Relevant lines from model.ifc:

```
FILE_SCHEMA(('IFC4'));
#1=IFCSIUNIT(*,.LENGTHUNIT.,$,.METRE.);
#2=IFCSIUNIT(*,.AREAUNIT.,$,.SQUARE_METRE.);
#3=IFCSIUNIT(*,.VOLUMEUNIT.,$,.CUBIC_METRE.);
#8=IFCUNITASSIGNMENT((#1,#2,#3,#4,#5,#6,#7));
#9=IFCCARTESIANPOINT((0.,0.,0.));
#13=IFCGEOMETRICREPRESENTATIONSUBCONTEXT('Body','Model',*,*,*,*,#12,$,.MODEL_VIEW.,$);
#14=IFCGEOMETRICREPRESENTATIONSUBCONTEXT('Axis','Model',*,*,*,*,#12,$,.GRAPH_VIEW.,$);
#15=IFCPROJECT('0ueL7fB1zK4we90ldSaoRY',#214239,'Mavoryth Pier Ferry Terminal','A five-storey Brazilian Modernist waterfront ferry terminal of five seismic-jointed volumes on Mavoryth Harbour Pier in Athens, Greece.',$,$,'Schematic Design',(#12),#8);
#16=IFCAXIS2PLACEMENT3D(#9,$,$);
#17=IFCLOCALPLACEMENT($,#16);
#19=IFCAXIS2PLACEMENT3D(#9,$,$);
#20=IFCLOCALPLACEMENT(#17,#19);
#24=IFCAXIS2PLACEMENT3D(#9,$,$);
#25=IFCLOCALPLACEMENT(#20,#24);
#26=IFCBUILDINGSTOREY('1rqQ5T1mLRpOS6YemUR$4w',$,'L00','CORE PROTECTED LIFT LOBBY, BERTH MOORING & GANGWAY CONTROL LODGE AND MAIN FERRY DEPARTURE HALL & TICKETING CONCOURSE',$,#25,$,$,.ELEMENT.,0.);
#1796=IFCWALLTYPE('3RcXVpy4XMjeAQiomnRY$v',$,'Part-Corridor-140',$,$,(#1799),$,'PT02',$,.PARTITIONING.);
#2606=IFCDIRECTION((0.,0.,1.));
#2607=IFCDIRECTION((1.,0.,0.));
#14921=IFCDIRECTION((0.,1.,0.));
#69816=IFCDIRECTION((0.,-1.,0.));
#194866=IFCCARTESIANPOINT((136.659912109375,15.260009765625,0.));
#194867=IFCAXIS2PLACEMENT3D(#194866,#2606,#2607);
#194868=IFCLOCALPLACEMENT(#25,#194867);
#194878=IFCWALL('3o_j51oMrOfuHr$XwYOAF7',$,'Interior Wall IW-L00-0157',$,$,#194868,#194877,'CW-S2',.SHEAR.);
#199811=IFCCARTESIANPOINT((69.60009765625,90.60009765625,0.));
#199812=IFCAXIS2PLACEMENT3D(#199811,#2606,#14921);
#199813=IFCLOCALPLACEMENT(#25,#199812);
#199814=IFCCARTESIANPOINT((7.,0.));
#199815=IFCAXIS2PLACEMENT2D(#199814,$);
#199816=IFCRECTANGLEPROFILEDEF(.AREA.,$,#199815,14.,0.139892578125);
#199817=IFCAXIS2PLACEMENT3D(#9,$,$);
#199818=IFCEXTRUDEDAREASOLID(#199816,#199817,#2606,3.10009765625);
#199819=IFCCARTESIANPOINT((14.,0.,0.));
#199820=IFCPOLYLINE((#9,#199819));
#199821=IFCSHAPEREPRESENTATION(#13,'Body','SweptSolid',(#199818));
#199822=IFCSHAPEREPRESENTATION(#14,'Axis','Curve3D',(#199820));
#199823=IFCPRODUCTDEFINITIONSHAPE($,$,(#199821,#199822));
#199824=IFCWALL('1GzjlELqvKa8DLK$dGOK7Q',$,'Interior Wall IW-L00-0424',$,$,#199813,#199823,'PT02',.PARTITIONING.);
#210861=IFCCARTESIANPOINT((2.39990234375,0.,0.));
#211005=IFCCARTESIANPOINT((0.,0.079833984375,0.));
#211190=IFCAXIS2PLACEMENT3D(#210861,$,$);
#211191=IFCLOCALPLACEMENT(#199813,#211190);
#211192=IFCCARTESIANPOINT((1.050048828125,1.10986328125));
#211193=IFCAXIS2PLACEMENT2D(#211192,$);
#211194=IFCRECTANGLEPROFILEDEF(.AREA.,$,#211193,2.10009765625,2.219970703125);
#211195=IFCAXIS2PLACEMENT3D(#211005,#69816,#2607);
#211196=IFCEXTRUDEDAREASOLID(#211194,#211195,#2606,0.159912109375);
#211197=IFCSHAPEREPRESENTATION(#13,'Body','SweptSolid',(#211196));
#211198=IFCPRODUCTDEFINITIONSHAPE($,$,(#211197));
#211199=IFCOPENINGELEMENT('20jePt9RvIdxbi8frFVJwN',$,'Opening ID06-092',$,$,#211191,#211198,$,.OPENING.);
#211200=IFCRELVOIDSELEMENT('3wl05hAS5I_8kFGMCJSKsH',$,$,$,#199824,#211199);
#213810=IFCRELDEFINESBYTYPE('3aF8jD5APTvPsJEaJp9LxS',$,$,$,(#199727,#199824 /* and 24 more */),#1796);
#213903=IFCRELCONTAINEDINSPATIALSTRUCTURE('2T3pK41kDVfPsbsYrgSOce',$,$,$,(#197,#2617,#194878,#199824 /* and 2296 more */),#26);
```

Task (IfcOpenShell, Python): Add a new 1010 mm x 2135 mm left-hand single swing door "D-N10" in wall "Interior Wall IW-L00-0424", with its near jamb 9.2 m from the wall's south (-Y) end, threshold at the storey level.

```python
import numpy as np
import ifcopenshell
import ifcopenshell.api.feature
import ifcopenshell.api.geometry
import ifcopenshell.api.root
import ifcopenshell.api.spatial
import ifcopenshell.geom
import ifcopenshell.util.element
import ifcopenshell.util.placement
import ifcopenshell.util.representation
import ifcopenshell.util.shape
import ifcopenshell.util.unit

model = ifcopenshell.open("model.ifc")
unit_scale = ifcopenshell.util.unit.calculate_unit_scale(model)
settings = ifcopenshell.geom.settings()


def volume(element):
    """Net volume in cubic metres, openings subtracted."""
    shape = ifcopenshell.geom.create_shape(settings, element)
    return ifcopenshell.util.shape.get_volume(shape.geometry)


wall = model.by_guid("1GzjlELqvKa8DLK$dGOK7Q")
storey = ifcopenshell.util.element.get_container(wall, ifc_class="IfcBuildingStorey")
context = ifcopenshell.util.representation.get_context(model, "Model", "Body", "MODEL_VIEW")
before = volume(wall)

width, height, from_end, sill = 1.01, 2.135, 9.2, 0.0  # metres

# The wall runs along its own X axis, and the end named is its -X end.
wall_shape = ifcopenshell.geom.create_shape(settings, wall)
x, y, z = ifcopenshell.util.shape.get_vertices(wall_shape.geometry).T
start = x.min() + from_end
face, thickness = float(y.min()), float(y.max() - y.min())
wall_matrix = ifcopenshell.util.placement.get_local_placement(wall.ObjectPlacement)
level = ifcopenshell.util.placement.get_local_placement(storey.ObjectPlacement)[2, 3]


def in_wall(x, y):
    """Placement at x, y metres in the wall's axes, at sill height."""
    matrix = wall_matrix.copy()
    matrix[:, 3] = wall_matrix @ np.array([x / unit_scale, y / unit_scale, 0.0, 1.0])
    matrix[2, 3] = level + sill / unit_scale
    return matrix


# Opening: a box that overshoots both wall faces by 50 mm.
opening = ifcopenshell.api.root.create_entity(model, ifc_class="IfcOpeningElement", predefined_type="OPENING")
box = ifcopenshell.api.geometry.add_wall_representation(
    model, context=context, length=width, height=height, thickness=thickness + 0.1
)
ifcopenshell.api.geometry.assign_representation(model, product=opening, representation=box)
ifcopenshell.api.geometry.edit_object_placement(model, product=opening, matrix=in_wall(start, face - 0.05), is_si=False)
ifcopenshell.api.feature.add_feature(model, feature=opening, element=wall)

door = ifcopenshell.api.root.create_entity(model, ifc_class="IfcDoor", name="D-N10", predefined_type="DOOR")
door.OverallWidth, door.OverallHeight = width / unit_scale, height / unit_scale
door.OperationType = "SINGLE_SWING_LEFT"
body = ifcopenshell.api.geometry.add_door_representation(
    model,
    context=context,
    overall_width=door.OverallWidth,
    overall_height=door.OverallHeight,
    operation_type="SINGLE_SWING_LEFT",
    lining_properties={"LiningDepth": thickness / unit_scale, "ThresholdDepth": thickness / unit_scale},
)
ifcopenshell.api.geometry.assign_representation(model, product=door, representation=body)
ifcopenshell.api.spatial.assign_container(model, products=[door], relating_structure=storey)
ifcopenshell.api.feature.add_filling(model, opening=opening, element=door)

# The lining spans the wall, so the door starts at the wall face.
ifcopenshell.api.geometry.edit_object_placement(model, product=door, matrix=in_wall(start, face), is_si=False)

after = volume(wall)

print(f"wall volume {before:.3f} -> {after:.3f} m3")

model.write("model_rev.ifc")
```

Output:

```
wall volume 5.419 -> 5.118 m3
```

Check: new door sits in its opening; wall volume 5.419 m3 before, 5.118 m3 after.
